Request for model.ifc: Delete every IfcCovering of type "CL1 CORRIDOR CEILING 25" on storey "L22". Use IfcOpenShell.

First a look at what the model holds.

```python
import ifcopenshell
import ifcopenshell.util.element

model = ifcopenshell.open("model.ifc")
print(model.schema)
storey = next(s for s in model.by_type("IfcBuildingStorey") if s.Name == "L22")
coverings = [e for e in ifcopenshell.util.element.get_decomposition(storey) if e.is_a("IfcCovering")]
seen = {}
for e in coverings:
    element_type = ifcopenshell.util.element.get_type(e)
    name = element_type.Name if element_type not in (None, e) else None
    seen[name] = seen.get(name, 0) + 1
for name, count in sorted(seen.items(), key=str):
    print(count, "x", name)
```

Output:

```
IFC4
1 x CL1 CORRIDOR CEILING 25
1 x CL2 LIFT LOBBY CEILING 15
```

```python
import ifcopenshell
import ifcopenshell.api.root
import ifcopenshell.util.element

model = ifcopenshell.open("model.ifc")

storey = next(s for s in model.by_type("IfcBuildingStorey") if s.Name == "L22")
coverings = [e for e in ifcopenshell.util.element.get_decomposition(storey) if e.is_a("IfcCovering")]
targets = [e for e in coverings if (t := ifcopenshell.util.element.get_type(e)) not in (None, e) and t.Name == "CL1 CORRIDOR CEILING 25"]

for e in targets:
    ifcopenshell.api.root.remove_product(model, product=e)
print(len(targets), "removed")

model.write("model_updated.ifc")
```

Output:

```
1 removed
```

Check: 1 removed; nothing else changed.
